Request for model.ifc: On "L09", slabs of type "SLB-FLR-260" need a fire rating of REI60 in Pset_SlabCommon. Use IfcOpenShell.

First a look at what the model holds.

```python
import ifcopenshell
import ifcopenshell.util.element

model = ifcopenshell.open("model.ifc")
print(model.schema)
storey = next(s for s in model.by_type("IfcBuildingStorey") if s.Name == "L09")
slabs = [e for e in ifcopenshell.util.element.get_decomposition(storey) if e.is_a("IfcSlab")]
seen = {}
for e in slabs:
    element_type = ifcopenshell.util.element.get_type(e)
    key = (element_type.Name if element_type != e and element_type else None, ifcopenshell.util.element.get_pset(e, "Pset_SlabCommon", "FireRating"))
    seen[key] = seen.get(key, 0) + 1
for (name, value), count in sorted(seen.items(), key=str):
    print(count, "x", name, "|", value)
```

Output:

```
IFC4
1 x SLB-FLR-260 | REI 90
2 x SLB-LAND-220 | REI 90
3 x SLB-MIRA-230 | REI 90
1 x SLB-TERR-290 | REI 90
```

```python
import ifcopenshell
import ifcopenshell.api.pset
import ifcopenshell.util.element

model = ifcopenshell.open("model.ifc")

storey = next(s for s in model.by_type("IfcBuildingStorey") if s.Name == "L09")
slabs = [e for e in ifcopenshell.util.element.get_decomposition(storey) if e.is_a("IfcSlab")]

count = 0
for e in slabs:
    element_type = ifcopenshell.util.element.get_type(e)
    if element_type in (None, e) or element_type.Name != "SLB-FLR-260":
        continue
    # add_pset returns the element's existing set when there is one.
    pset = ifcopenshell.api.pset.add_pset(model, product=e, name="Pset_SlabCommon")
    ifcopenshell.api.pset.edit_pset(model, pset=pset, properties={"FireRating": "REI60"})
    count += 1

print(count, "slabs updated")

model.write("model_rev.ifc")
```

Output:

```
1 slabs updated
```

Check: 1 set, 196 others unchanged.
